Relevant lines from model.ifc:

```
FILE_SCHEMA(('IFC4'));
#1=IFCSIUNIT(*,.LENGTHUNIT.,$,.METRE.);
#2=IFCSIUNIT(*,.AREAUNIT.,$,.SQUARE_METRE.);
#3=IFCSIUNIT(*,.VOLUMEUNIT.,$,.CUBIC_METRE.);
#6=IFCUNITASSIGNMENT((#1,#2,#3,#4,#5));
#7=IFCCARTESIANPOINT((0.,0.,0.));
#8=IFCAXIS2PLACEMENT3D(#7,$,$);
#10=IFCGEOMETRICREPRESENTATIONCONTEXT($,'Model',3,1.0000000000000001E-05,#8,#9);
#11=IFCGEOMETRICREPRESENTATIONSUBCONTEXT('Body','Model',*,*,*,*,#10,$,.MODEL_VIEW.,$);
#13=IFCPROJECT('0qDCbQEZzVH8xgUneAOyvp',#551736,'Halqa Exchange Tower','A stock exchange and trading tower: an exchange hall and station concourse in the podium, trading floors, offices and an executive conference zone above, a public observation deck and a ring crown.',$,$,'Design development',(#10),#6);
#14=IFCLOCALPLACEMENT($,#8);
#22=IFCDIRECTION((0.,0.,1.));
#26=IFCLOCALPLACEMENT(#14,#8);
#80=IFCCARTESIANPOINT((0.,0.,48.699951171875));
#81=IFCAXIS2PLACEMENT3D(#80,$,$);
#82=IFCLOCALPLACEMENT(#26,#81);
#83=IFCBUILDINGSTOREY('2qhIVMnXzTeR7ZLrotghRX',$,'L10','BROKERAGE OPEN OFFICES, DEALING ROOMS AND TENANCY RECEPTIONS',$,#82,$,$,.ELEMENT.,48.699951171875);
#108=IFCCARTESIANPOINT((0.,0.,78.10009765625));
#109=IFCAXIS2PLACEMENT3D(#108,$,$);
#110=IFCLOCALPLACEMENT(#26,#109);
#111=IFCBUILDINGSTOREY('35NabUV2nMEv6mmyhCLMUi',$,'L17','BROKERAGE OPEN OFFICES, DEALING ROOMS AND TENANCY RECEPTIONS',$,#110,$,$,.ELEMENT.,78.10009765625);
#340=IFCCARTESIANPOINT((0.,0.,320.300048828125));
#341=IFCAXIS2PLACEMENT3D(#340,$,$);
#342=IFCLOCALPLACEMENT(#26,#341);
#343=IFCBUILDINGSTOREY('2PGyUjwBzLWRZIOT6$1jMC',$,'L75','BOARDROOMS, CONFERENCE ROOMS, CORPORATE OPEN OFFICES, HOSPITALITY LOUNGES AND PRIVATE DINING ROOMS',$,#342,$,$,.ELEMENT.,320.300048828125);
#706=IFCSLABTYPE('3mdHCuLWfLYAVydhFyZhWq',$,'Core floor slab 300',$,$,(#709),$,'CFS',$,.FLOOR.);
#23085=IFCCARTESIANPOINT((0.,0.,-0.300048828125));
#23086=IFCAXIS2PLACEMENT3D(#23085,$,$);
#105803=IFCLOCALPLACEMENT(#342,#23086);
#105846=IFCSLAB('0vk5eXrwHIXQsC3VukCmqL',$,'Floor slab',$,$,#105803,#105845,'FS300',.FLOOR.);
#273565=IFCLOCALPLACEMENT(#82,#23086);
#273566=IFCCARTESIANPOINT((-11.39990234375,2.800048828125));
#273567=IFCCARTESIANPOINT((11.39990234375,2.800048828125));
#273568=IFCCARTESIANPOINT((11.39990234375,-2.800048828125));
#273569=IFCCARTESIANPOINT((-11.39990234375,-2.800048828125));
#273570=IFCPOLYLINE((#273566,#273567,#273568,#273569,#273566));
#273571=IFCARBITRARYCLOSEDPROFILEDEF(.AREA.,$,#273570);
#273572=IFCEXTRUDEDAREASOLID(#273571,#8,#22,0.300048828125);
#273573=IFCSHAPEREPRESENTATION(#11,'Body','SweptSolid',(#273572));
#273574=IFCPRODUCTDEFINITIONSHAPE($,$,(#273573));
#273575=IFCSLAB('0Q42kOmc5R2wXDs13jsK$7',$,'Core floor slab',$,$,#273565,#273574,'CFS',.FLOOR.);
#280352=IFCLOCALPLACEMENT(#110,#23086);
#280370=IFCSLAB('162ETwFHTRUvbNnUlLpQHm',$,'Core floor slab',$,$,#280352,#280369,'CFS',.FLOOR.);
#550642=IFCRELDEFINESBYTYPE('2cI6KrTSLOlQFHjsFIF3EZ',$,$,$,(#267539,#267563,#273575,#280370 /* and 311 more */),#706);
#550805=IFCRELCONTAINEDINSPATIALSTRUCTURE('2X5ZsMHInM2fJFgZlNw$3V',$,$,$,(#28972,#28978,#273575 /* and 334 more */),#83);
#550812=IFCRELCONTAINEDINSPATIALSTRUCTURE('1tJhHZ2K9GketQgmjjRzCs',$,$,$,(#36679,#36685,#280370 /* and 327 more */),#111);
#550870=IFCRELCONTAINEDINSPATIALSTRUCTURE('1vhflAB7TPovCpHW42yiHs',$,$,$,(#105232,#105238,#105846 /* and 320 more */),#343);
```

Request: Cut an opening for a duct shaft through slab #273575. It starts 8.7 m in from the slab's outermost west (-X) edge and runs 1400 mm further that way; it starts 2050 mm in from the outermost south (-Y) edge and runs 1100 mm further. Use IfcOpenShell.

```python
import numpy as np
import ifcopenshell
import ifcopenshell.api.feature
import ifcopenshell.api.geometry
import ifcopenshell.api.root
import ifcopenshell.geom
import ifcopenshell.util.placement
import ifcopenshell.util.representation
import ifcopenshell.util.shape
import ifcopenshell.util.unit

model = ifcopenshell.open("model.ifc")
unit_scale = ifcopenshell.util.unit.calculate_unit_scale(model)
settings = ifcopenshell.geom.settings()


def volume(element):
    """Net volume in cubic metres, openings subtracted."""
    shape = ifcopenshell.geom.create_shape(settings, element)
    return ifcopenshell.util.shape.get_volume(shape.geometry)


slab = model.by_id(273575)
before = volume(slab)

# Extent in the slab's own axes, in metres. The edges named are its -X and -Y sides.
slab_shape = ifcopenshell.geom.create_shape(settings, slab)
vertices = ifcopenshell.util.shape.get_vertices(slab_shape.geometry)
x_min, y_min, bottom = vertices.min(axis=0)
top = vertices[:, 2].max()

opening = ifcopenshell.api.root.create_entity(model, ifc_class="IfcOpeningElement", name="Duct shaft opening", predefined_type="OPENING")
context = ifcopenshell.util.representation.get_context(model, "Model", "Body", "MODEL_VIEW")
width, depth = 1.4, 1.1
outline = [(0.0, 0.0), (width, 0.0), (width, depth), (0.0, depth), (0.0, 0.0)]
# Overshoot both faces by 50 mm so the cut is clean.
shape = ifcopenshell.api.geometry.add_slab_representation(
    model, context=context, depth=top - bottom + 0.1, polyline=outline
)
ifcopenshell.api.geometry.assign_representation(model, product=opening, representation=shape)

matrix = ifcopenshell.util.placement.get_local_placement(slab.ObjectPlacement)
matrix[:, 3] = matrix @ np.append(np.array([x_min + 8.7, y_min + 2.05, bottom - 0.05]) / unit_scale, 1.0)
ifcopenshell.api.geometry.edit_object_placement(model, product=opening, matrix=matrix, is_si=False)
ifcopenshell.api.feature.add_feature(model, feature=opening, element=slab)

after = volume(slab)

print(f"slab volume {before:.3f} -> {after:.3f} m3")

model.write("model_rev.ifc")
```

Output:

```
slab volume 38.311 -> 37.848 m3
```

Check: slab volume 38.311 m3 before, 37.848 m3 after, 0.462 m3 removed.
